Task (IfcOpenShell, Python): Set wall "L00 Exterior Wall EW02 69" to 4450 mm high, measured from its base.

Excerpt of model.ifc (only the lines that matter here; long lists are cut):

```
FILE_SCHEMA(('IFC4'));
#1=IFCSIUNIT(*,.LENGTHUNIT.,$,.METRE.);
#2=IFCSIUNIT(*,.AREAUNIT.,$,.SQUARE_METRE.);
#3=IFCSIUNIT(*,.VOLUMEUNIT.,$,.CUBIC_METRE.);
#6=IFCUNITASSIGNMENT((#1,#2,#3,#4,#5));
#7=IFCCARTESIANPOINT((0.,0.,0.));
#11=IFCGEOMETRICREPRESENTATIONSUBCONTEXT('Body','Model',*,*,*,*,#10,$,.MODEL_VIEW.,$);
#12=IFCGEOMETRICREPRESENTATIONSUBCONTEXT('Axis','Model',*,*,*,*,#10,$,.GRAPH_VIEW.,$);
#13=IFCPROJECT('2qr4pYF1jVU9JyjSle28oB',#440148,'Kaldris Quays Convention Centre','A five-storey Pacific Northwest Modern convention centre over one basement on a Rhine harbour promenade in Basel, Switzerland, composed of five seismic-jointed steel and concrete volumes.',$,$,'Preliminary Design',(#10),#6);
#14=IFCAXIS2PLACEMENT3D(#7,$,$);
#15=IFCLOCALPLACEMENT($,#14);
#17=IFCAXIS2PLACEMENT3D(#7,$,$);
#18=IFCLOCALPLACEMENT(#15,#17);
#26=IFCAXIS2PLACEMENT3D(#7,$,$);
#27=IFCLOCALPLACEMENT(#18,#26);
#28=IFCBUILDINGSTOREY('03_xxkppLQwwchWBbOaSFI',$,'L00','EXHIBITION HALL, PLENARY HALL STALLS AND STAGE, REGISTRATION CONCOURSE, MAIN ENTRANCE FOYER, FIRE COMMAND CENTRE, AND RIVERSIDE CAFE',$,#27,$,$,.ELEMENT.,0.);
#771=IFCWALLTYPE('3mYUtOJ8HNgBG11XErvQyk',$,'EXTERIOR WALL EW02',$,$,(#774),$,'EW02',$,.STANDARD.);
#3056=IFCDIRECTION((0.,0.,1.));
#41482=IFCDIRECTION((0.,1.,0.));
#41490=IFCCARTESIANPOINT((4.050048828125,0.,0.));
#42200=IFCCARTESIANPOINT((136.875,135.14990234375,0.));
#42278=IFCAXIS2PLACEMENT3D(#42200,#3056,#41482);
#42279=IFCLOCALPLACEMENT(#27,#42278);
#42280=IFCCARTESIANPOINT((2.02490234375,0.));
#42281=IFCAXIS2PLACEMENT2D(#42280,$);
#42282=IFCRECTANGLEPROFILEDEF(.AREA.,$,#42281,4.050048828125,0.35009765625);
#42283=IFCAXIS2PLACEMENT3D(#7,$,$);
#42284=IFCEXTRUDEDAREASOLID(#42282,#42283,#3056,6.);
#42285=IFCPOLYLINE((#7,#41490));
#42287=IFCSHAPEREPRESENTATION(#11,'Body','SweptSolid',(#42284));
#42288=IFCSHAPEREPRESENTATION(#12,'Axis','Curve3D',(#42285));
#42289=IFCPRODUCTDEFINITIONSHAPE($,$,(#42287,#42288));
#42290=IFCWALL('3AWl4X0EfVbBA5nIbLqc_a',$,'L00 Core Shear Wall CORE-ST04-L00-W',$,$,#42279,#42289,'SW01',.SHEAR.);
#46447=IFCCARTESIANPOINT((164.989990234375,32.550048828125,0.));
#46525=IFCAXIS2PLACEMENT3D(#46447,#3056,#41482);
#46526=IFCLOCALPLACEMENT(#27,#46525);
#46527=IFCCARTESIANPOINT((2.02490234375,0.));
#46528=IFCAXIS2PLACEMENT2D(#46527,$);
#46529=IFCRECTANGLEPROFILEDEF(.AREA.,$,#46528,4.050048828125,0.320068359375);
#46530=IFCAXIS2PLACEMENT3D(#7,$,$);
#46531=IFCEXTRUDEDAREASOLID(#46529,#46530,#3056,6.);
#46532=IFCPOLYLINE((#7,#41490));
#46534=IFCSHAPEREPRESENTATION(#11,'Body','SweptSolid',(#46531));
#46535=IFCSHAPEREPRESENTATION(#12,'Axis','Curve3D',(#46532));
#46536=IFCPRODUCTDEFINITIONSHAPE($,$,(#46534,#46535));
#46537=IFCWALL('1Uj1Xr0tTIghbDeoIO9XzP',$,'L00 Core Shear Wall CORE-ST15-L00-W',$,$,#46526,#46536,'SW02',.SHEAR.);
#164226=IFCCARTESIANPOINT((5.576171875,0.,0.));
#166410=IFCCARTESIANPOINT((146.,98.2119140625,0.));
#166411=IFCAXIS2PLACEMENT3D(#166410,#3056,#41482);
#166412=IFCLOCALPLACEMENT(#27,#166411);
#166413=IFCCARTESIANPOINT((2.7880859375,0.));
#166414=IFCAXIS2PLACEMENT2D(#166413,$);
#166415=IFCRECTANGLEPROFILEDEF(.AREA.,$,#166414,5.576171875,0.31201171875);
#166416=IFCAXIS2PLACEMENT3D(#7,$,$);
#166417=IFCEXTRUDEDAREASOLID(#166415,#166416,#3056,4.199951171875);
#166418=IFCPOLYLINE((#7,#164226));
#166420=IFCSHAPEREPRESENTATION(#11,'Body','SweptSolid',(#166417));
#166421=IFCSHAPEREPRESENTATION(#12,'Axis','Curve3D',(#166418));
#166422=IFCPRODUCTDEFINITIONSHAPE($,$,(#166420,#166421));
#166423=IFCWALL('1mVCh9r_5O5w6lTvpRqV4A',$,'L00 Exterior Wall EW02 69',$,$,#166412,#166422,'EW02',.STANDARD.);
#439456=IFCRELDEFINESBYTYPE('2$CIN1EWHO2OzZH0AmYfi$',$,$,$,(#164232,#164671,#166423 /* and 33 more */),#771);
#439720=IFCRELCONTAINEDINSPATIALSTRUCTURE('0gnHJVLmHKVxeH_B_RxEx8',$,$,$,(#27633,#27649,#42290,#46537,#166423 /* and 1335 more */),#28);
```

```python
import ifcopenshell
import ifcopenshell.geom
import ifcopenshell.util.representation
import ifcopenshell.util.shape
import ifcopenshell.util.unit

model = ifcopenshell.open("model.ifc")
unit_scale = ifcopenshell.util.unit.calculate_unit_scale(model)
settings = ifcopenshell.geom.settings()


def volume(element):
    """Net volume in cubic metres, openings subtracted."""
    shape = ifcopenshell.geom.create_shape(settings, element)
    return ifcopenshell.util.shape.get_volume(shape.geometry)


wall = model.by_id(166423)
before = volume(wall)

body = ifcopenshell.util.representation.get_representation(wall, "Model", "Body")
solid = body.Items[0]
old_height = solid.Depth
solid.Depth = 4.45 / unit_scale
after = volume(wall)

print(f"height {old_height:g} -> {solid.Depth:g}, volume {before:.3f} -> {after:.3f} m3")

model.write("model_v2.ifc")
```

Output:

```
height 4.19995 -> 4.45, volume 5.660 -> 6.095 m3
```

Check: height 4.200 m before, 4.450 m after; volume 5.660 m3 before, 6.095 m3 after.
